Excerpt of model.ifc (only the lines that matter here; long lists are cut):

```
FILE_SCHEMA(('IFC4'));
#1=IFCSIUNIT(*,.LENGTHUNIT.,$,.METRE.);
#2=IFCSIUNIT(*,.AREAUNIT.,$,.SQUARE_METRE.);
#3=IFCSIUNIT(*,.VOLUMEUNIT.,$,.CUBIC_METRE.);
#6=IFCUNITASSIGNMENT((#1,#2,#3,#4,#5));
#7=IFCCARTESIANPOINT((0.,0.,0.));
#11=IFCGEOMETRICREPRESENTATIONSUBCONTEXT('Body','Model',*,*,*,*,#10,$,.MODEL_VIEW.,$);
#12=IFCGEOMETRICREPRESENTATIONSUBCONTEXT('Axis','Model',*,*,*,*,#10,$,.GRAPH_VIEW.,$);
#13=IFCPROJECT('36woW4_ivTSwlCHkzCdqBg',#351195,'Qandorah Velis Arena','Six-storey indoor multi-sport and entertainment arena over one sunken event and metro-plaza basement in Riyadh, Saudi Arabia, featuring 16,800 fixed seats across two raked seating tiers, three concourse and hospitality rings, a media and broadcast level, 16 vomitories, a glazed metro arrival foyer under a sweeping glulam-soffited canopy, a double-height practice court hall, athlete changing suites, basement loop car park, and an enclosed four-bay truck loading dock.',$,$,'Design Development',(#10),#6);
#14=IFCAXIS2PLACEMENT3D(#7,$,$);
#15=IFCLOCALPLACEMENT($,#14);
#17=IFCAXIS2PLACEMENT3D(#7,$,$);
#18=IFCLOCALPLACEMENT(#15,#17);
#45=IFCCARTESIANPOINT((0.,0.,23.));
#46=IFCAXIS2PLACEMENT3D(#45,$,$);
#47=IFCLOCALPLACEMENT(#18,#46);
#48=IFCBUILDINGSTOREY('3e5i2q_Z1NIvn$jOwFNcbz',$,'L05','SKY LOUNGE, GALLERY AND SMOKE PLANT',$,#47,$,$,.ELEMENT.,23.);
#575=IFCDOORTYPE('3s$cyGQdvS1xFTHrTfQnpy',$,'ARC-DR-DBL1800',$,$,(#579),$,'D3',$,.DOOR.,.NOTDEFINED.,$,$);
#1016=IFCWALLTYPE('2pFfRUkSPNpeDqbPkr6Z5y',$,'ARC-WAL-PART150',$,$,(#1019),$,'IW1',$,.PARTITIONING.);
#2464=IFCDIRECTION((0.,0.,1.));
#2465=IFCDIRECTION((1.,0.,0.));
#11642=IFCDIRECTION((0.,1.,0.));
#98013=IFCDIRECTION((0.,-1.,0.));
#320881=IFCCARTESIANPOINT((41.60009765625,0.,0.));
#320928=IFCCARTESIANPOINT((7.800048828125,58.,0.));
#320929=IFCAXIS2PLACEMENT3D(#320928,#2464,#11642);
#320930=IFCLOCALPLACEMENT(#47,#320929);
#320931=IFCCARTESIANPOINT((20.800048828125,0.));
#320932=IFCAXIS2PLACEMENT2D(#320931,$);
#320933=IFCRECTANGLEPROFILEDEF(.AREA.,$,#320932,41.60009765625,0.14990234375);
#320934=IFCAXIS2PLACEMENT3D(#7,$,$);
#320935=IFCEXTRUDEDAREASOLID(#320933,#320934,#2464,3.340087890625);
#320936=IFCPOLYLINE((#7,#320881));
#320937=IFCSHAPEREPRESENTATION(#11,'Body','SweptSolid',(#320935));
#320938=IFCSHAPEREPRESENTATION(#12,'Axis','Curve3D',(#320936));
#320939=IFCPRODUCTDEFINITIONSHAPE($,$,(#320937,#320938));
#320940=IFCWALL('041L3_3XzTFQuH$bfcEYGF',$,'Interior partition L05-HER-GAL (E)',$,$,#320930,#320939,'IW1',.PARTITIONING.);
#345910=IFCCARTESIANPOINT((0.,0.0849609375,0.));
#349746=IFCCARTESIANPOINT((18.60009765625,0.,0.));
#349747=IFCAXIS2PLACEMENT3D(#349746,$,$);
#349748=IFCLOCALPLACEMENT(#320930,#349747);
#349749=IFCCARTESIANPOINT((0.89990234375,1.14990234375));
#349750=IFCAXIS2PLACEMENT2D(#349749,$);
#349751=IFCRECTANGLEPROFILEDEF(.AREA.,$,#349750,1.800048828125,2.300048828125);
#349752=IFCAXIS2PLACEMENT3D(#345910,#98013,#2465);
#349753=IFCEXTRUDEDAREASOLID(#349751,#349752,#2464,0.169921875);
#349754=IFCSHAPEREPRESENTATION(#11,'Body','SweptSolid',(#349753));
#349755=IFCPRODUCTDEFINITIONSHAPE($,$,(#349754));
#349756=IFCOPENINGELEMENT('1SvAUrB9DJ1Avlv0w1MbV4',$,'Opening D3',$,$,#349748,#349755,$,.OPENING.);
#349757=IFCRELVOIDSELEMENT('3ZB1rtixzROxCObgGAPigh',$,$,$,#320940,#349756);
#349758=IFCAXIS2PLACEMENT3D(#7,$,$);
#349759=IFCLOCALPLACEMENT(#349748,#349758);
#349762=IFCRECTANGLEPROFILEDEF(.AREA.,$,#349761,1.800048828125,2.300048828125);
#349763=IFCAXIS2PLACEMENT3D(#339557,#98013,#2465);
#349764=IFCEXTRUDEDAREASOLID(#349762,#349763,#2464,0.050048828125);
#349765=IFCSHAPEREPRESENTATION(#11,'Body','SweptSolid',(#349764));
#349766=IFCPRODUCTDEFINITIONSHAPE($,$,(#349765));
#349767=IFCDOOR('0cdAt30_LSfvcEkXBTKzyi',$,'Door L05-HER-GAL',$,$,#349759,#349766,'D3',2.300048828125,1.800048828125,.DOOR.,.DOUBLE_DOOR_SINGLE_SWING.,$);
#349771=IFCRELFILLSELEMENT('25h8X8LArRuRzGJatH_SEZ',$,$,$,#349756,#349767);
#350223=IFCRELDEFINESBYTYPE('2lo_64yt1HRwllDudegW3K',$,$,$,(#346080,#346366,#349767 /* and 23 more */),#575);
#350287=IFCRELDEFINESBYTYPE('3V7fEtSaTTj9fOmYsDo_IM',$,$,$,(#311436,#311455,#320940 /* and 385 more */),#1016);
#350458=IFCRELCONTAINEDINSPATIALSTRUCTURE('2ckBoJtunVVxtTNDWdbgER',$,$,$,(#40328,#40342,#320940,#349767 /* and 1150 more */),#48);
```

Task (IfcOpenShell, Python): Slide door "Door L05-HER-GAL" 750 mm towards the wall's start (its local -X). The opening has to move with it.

```python
import ifcopenshell
import ifcopenshell.api.geometry
import ifcopenshell.util.placement
import ifcopenshell.util.unit

model = ifcopenshell.open("model.ifc")
unit_scale = ifcopenshell.util.unit.calculate_unit_scale(model)

door = model.by_guid("0cdAt30_LSfvcEkXBTKzyi")
opening = door.FillsVoids[0].RelatingOpeningElement
wall = opening.VoidsElements[0].RelatingBuildingElement

wall_matrix = ifcopenshell.util.placement.get_local_placement(wall.ObjectPlacement)
shift = wall_matrix[:3, 0] * -0.75 / unit_scale
before = ifcopenshell.util.placement.get_local_placement(door.ObjectPlacement)[:3, 3].copy()

# The door is placed relative to its opening, so it follows when the opening moves.
matrix = ifcopenshell.util.placement.get_local_placement(opening.ObjectPlacement)
matrix[:3, 3] += shift
ifcopenshell.api.geometry.edit_object_placement(
    model, product=opening, matrix=matrix, is_si=False, should_transform_children=True
)

after = ifcopenshell.util.placement.get_local_placement(door.ObjectPlacement)[:3, 3]
print("door moved by", (after - before).round(3) + 0.0)

model.write("model_v2.ifc")
```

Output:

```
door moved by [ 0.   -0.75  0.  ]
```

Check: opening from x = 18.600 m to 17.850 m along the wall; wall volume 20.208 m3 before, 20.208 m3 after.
